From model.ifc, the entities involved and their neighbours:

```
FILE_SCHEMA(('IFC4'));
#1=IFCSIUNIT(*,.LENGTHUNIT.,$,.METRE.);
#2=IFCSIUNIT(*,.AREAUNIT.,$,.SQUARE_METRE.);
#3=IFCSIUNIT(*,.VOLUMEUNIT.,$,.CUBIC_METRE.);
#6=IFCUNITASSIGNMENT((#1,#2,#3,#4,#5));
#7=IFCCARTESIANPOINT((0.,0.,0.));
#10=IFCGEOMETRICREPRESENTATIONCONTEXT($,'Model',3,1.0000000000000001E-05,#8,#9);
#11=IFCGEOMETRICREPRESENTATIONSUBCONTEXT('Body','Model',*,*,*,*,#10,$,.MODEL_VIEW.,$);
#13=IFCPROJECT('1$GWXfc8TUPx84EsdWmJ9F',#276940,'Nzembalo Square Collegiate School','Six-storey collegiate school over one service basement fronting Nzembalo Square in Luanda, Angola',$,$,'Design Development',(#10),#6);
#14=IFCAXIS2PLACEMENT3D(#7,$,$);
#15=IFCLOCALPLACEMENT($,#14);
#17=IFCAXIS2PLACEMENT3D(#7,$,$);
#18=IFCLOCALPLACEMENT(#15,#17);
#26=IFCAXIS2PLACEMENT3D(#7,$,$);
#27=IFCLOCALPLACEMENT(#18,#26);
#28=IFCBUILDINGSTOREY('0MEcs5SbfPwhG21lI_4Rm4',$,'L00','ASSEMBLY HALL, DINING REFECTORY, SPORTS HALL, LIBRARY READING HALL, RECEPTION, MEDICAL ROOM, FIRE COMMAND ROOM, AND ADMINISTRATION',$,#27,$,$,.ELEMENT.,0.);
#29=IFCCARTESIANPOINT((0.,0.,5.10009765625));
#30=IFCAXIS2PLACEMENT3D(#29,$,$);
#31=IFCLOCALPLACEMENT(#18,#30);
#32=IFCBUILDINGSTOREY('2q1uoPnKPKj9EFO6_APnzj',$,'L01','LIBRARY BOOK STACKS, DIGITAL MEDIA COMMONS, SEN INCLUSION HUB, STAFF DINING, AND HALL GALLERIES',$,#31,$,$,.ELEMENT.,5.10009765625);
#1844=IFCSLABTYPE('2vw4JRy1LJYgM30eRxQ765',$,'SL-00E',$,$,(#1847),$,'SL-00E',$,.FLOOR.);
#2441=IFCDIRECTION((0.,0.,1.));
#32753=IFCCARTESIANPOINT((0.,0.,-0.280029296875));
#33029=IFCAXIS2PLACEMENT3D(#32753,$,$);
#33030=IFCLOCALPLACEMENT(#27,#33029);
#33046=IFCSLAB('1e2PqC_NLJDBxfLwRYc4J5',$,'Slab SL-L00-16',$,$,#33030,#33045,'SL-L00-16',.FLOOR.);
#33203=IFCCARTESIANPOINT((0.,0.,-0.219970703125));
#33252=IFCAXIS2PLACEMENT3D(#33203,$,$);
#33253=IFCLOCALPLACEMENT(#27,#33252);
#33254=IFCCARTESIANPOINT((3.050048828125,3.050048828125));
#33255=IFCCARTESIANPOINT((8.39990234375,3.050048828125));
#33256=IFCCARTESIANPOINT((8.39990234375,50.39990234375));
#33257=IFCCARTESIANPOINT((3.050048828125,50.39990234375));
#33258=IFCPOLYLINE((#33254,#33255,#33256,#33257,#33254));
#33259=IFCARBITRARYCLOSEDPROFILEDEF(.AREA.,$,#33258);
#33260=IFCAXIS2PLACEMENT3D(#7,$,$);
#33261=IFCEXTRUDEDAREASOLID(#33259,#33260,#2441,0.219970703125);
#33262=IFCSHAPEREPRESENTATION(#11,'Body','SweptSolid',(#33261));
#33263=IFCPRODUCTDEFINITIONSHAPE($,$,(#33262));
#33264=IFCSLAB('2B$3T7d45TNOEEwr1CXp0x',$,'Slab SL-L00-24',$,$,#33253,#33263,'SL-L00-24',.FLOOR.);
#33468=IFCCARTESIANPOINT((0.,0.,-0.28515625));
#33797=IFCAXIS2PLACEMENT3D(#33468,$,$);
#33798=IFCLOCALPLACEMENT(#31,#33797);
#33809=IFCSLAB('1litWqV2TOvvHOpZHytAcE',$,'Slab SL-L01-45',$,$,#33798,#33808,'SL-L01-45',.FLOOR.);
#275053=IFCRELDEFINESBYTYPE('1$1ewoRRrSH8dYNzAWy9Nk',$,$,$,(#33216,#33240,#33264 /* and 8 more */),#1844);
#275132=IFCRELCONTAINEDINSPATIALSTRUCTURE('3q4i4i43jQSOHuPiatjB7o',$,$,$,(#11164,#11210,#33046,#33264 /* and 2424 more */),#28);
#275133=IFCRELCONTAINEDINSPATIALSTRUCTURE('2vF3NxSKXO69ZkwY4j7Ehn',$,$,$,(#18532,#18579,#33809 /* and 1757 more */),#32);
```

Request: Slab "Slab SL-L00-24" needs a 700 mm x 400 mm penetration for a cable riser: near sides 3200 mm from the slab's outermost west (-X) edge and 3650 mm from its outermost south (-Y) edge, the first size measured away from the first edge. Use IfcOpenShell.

```python
import numpy as np
import ifcopenshell
import ifcopenshell.api.feature
import ifcopenshell.api.geometry
import ifcopenshell.api.root
import ifcopenshell.geom
import ifcopenshell.util.placement
import ifcopenshell.util.representation
import ifcopenshell.util.shape
import ifcopenshell.util.unit

model = ifcopenshell.open("model.ifc")
unit_scale = ifcopenshell.util.unit.calculate_unit_scale(model)
settings = ifcopenshell.geom.settings()


def volume(element):
    """Net volume in cubic metres, openings subtracted."""
    shape = ifcopenshell.geom.create_shape(settings, element)
    return ifcopenshell.util.shape.get_volume(shape.geometry)


slab = model.by_guid("2B$3T7d45TNOEEwr1CXp0x")
before = volume(slab)

# Extent in the slab's own axes, in metres. The edges named are its -X and -Y sides.
slab_shape = ifcopenshell.geom.create_shape(settings, slab)
vertices = ifcopenshell.util.shape.get_vertices(slab_shape.geometry)
x_min, y_min, bottom = vertices.min(axis=0)
top = vertices[:, 2].max()

opening = ifcopenshell.api.root.create_entity(model, ifc_class="IfcOpeningElement", name="Cable riser opening", predefined_type="OPENING")
context = ifcopenshell.util.representation.get_context(model, "Model", "Body", "MODEL_VIEW")
width, depth = 0.7, 0.4
outline = [(0.0, 0.0), (width, 0.0), (width, depth), (0.0, depth), (0.0, 0.0)]
# Overshoot both faces by 50 mm so the cut is clean.
shape = ifcopenshell.api.geometry.add_slab_representation(
    model, context=context, depth=top - bottom + 0.1, polyline=outline
)
ifcopenshell.api.geometry.assign_representation(model, product=opening, representation=shape)

matrix = ifcopenshell.util.placement.get_local_placement(slab.ObjectPlacement)
matrix[:, 3] = matrix @ np.append(np.array([x_min + 3.2, y_min + 3.65, bottom - 0.05]) / unit_scale, 1.0)
ifcopenshell.api.geometry.edit_object_placement(model, product=opening, matrix=matrix, is_si=False)
ifcopenshell.api.feature.add_feature(model, feature=opening, element=slab)

after = volume(slab)

print(f"slab volume {before:.3f} -> {after:.3f} m3")

model.write("model-out.ifc")
```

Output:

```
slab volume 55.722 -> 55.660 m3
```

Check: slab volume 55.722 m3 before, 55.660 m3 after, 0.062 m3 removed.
